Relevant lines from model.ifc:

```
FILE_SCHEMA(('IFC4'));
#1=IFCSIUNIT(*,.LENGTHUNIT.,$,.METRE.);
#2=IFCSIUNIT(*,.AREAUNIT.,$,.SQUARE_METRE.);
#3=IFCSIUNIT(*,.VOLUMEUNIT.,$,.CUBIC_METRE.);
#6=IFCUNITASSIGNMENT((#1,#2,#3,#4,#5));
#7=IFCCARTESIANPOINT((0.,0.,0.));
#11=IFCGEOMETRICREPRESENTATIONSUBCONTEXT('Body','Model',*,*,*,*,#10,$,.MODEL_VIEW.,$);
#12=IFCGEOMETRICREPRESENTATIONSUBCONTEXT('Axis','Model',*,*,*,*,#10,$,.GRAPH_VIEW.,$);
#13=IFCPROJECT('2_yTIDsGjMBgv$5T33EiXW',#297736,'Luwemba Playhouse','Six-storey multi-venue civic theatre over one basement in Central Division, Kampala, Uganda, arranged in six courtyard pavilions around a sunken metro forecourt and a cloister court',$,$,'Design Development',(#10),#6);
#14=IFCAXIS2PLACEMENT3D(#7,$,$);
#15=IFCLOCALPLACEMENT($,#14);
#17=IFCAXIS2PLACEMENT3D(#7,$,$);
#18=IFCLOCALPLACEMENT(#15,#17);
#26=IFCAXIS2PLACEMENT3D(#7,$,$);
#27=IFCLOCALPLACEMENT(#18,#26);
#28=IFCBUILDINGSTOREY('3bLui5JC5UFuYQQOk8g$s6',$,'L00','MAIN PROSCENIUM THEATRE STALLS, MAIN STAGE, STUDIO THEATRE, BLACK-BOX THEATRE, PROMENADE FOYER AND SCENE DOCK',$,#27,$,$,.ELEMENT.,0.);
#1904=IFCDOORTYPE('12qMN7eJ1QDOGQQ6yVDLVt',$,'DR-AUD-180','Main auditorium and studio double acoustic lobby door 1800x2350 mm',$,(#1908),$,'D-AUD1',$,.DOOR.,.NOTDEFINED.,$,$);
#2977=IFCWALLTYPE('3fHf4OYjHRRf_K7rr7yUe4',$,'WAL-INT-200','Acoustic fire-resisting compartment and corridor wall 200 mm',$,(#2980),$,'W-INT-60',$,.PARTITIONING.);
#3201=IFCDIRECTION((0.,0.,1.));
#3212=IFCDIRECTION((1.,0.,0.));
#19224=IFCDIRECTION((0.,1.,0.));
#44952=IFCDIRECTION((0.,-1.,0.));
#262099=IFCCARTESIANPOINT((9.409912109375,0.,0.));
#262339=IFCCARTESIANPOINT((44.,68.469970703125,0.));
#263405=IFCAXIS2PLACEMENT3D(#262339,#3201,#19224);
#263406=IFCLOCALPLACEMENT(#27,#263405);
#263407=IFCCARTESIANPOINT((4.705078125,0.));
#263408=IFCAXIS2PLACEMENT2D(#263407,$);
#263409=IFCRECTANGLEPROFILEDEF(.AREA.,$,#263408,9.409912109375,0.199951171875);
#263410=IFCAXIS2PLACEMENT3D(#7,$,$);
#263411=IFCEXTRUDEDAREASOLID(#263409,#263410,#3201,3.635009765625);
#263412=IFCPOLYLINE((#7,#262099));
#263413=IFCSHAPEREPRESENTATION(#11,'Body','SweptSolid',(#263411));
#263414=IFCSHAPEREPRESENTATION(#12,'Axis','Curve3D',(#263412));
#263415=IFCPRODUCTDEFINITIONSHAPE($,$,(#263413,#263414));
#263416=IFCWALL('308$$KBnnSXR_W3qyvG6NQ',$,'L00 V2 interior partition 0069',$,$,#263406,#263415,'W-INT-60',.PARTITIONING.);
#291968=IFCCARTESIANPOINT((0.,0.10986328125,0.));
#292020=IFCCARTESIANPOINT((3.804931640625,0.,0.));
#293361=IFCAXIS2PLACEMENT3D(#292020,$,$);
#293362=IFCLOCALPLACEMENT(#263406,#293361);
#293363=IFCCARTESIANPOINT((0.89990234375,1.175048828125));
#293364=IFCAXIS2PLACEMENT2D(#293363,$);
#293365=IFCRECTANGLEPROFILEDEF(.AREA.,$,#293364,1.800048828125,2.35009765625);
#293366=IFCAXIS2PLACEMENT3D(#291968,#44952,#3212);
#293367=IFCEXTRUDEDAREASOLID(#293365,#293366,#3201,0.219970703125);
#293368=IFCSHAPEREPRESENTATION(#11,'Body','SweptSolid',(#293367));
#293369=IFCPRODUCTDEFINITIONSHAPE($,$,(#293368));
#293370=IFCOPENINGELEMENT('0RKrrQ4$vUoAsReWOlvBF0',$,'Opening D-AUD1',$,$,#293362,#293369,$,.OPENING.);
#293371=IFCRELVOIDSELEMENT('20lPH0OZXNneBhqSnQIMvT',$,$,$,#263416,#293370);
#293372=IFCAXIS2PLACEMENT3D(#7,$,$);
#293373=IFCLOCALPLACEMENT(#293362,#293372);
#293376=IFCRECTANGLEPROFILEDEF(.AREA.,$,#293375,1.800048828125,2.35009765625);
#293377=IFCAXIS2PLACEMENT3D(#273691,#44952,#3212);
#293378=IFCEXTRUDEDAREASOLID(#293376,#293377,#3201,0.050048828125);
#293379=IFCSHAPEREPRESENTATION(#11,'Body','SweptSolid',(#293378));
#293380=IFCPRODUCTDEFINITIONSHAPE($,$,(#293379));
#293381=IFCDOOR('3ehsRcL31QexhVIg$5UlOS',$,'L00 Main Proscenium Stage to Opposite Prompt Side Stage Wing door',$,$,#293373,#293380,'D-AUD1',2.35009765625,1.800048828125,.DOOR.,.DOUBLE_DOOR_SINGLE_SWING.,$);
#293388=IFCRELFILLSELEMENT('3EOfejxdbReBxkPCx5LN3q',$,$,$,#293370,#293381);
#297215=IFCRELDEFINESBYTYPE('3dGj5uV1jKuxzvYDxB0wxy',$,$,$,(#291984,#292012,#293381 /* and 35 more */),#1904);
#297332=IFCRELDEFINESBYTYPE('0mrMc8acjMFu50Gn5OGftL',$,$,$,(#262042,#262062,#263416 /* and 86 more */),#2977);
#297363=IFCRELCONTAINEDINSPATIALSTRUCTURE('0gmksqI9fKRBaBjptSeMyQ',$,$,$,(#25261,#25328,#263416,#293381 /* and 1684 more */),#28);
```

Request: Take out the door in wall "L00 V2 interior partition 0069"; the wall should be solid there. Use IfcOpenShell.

```python
import ifcopenshell
import ifcopenshell.api.feature
import ifcopenshell.api.root
import ifcopenshell.geom
import ifcopenshell.util.shape

model = ifcopenshell.open("model.ifc")
settings = ifcopenshell.geom.settings()


def volume(element):
    """Net volume in cubic metres, openings subtracted."""
    shape = ifcopenshell.geom.create_shape(settings, element)
    return ifcopenshell.util.shape.get_volume(shape.geometry)


door = model.by_guid("3ehsRcL31QexhVIg$5UlOS")
opening = door.FillsVoids[0].RelatingOpeningElement
wall = opening.VoidsElements[0].RelatingBuildingElement
before = volume(wall)

ifcopenshell.api.root.remove_product(model, product=door)
ifcopenshell.api.feature.remove_feature(model, feature=opening)

after = volume(wall)

print(f"wall volume {before:.3f} -> {after:.3f} m3")

model.write("model_rev.ifc")
```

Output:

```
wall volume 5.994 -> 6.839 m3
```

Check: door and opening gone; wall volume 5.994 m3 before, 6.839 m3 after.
